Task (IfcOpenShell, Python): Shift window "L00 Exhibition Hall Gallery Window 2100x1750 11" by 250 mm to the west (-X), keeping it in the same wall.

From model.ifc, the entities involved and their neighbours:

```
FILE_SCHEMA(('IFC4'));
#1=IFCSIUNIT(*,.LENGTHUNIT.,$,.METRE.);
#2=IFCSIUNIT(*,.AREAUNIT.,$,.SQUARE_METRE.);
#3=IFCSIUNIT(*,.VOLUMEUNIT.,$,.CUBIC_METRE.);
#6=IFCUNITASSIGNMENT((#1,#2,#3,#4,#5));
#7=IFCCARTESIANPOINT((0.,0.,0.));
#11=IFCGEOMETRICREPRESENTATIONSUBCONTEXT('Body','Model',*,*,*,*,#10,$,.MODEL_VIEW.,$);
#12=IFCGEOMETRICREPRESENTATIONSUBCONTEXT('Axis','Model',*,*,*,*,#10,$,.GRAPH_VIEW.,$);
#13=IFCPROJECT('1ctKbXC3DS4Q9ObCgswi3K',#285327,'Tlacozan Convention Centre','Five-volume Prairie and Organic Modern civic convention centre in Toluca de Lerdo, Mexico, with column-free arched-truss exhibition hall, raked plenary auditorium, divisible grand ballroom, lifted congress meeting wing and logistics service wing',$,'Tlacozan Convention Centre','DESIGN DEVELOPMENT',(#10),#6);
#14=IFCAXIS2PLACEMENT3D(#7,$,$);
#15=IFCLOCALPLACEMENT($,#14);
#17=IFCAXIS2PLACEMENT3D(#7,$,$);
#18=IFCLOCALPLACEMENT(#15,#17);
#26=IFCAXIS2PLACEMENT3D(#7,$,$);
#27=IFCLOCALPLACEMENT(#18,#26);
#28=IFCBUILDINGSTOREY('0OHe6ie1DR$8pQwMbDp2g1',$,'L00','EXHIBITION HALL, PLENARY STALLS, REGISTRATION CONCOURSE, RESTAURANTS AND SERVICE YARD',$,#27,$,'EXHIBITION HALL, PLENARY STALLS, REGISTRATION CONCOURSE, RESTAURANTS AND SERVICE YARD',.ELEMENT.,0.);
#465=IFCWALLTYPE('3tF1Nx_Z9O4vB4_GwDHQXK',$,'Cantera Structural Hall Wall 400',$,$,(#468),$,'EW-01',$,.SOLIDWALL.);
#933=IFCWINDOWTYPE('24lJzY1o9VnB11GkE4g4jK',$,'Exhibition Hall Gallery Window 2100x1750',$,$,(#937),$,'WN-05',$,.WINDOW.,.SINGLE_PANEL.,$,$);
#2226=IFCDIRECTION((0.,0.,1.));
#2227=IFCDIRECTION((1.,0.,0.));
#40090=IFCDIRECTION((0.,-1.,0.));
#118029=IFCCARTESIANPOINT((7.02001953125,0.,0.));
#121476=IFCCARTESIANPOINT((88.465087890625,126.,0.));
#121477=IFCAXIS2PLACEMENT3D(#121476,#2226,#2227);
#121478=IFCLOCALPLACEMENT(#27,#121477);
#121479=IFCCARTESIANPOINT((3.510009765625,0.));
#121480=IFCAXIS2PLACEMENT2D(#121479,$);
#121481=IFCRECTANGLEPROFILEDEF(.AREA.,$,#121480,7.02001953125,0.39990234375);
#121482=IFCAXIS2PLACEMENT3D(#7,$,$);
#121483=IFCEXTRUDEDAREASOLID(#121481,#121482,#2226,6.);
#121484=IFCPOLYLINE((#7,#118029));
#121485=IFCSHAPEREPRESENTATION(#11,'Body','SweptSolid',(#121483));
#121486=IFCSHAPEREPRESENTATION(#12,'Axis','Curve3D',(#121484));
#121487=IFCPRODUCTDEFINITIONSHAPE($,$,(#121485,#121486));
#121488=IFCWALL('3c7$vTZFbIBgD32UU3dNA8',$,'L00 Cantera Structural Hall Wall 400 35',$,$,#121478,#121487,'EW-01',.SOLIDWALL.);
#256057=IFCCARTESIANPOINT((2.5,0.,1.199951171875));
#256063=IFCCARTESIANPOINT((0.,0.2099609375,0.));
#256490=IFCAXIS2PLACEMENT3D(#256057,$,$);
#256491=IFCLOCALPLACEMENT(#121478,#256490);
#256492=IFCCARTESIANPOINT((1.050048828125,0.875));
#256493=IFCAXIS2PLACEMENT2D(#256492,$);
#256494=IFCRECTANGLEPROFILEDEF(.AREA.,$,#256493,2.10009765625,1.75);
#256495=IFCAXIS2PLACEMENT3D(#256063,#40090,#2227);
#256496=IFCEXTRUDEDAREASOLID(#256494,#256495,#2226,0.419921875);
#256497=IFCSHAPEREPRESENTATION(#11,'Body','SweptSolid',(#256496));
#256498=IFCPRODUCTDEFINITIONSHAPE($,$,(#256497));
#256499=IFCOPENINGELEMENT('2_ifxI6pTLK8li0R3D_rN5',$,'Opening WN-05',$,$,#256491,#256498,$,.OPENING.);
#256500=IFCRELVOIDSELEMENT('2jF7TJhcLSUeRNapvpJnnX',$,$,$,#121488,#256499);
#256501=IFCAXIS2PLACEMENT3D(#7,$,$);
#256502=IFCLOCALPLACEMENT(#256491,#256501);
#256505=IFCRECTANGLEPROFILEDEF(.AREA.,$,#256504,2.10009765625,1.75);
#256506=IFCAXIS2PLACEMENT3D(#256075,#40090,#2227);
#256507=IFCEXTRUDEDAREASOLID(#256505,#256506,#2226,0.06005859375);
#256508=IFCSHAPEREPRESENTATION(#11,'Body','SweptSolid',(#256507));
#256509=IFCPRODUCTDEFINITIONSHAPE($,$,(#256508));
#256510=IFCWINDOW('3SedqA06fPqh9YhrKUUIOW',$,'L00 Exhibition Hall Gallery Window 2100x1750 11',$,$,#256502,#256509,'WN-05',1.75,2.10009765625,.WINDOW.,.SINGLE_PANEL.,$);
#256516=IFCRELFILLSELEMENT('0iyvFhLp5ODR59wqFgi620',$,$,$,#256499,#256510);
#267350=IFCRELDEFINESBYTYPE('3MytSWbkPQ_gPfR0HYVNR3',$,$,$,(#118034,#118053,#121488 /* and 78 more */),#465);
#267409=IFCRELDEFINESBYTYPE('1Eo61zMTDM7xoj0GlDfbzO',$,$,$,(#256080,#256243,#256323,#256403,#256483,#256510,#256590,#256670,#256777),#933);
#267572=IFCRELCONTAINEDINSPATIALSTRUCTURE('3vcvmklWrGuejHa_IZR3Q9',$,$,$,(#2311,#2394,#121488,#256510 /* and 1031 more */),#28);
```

```python
import ifcopenshell
import ifcopenshell.api.geometry
import ifcopenshell.util.placement

model = ifcopenshell.open("model.ifc")

window = model.by_guid("3SedqA06fPqh9YhrKUUIOW")
opening = window.FillsVoids[0].RelatingOpeningElement
wall = opening.VoidsElements[0].RelatingBuildingElement

wall_matrix = ifcopenshell.util.placement.get_local_placement(wall.ObjectPlacement)
shift = wall_matrix[:3, 0] * -0.25
before = ifcopenshell.util.placement.get_local_placement(window.ObjectPlacement)[:3, 3].copy()

# The window is placed relative to its opening, so it follows when the opening moves.
matrix = ifcopenshell.util.placement.get_local_placement(opening.ObjectPlacement)
matrix[:3, 3] += shift
ifcopenshell.api.geometry.edit_object_placement(
    model, product=opening, matrix=matrix, is_si=False, should_transform_children=True
)

after = ifcopenshell.util.placement.get_local_placement(window.ObjectPlacement)[:3, 3]
print("window moved by", (after - before).round(3) + 0.0)

model.write("model_v2.ifc")
```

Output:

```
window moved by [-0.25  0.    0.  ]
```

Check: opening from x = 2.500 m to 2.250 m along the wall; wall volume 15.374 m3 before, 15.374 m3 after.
